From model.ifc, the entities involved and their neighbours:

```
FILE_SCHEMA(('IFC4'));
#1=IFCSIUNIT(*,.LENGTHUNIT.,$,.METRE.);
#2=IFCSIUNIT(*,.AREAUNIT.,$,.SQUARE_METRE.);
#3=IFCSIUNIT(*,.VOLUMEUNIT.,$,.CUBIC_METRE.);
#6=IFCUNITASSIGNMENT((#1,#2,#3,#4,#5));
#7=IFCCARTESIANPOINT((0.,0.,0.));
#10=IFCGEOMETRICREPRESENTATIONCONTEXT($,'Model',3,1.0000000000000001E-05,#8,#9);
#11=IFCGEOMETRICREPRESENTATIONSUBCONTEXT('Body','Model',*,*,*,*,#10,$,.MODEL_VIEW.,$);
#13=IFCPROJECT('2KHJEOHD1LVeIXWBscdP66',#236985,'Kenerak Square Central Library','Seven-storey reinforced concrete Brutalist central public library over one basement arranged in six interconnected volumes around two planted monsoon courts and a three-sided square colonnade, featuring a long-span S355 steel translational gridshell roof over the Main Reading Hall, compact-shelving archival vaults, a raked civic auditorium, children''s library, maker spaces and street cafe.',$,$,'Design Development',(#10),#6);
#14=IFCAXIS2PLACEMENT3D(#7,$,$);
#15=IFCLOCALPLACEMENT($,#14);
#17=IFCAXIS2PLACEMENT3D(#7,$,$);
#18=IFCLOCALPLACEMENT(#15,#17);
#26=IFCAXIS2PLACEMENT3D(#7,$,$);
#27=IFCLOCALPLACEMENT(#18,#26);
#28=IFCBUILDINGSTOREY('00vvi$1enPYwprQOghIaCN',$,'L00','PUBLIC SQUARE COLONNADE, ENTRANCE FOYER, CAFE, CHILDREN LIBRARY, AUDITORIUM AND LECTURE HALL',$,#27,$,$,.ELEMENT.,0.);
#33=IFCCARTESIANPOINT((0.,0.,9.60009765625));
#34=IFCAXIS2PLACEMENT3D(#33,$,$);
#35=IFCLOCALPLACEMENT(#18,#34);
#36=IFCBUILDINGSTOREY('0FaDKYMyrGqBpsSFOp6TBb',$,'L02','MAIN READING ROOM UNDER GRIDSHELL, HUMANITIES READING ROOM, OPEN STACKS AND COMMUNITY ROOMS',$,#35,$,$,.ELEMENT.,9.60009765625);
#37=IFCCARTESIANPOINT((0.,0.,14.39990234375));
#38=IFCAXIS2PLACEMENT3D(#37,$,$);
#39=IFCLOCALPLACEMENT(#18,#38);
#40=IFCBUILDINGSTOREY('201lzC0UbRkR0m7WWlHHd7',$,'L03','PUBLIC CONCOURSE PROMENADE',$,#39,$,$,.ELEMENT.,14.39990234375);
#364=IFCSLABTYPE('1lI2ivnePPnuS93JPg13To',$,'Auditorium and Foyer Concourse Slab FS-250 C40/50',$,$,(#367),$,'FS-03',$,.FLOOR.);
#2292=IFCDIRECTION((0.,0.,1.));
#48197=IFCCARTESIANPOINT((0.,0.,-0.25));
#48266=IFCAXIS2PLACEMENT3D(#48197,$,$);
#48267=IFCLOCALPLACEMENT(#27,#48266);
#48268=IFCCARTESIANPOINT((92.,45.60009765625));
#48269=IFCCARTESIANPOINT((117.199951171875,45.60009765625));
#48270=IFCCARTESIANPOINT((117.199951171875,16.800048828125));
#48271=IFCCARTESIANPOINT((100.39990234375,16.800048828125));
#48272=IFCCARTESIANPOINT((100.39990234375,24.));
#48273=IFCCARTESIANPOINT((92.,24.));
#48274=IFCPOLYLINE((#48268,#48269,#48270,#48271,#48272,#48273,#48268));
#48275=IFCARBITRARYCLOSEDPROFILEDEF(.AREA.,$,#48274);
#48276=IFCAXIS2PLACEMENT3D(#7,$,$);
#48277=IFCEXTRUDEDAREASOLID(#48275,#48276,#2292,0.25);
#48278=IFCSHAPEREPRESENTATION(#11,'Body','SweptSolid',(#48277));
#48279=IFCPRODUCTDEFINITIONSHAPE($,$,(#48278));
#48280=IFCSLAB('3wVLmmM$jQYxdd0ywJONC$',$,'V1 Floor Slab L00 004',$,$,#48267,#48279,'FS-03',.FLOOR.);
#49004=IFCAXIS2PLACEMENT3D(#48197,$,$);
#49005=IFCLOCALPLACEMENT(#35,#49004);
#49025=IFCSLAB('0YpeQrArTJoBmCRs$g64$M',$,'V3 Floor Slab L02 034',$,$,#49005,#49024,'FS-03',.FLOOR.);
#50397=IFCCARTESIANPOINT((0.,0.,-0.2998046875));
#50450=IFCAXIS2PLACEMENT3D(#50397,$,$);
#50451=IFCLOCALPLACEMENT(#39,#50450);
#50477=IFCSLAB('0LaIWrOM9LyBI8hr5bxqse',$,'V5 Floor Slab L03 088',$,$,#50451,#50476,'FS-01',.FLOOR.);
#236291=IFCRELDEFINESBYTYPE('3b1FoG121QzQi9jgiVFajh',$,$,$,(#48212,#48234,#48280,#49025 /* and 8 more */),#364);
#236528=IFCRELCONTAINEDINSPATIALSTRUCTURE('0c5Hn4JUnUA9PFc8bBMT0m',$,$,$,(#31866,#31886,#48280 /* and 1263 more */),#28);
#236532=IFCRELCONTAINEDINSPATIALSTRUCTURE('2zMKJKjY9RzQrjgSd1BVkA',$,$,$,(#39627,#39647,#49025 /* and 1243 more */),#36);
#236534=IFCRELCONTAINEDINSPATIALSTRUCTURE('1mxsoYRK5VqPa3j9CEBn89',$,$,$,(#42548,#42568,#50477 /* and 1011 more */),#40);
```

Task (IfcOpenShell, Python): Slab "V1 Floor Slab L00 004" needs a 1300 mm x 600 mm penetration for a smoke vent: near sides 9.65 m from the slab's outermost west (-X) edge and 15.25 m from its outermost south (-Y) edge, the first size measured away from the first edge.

```python
import numpy as np
import ifcopenshell
import ifcopenshell.api.feature
import ifcopenshell.api.geometry
import ifcopenshell.api.root
import ifcopenshell.geom
import ifcopenshell.util.placement
import ifcopenshell.util.representation
import ifcopenshell.util.shape
import ifcopenshell.util.unit

model = ifcopenshell.open("model.ifc")
unit_scale = ifcopenshell.util.unit.calculate_unit_scale(model)
settings = ifcopenshell.geom.settings()


def volume(element):
    """Net volume in cubic metres, openings subtracted."""
    shape = ifcopenshell.geom.create_shape(settings, element)
    return ifcopenshell.util.shape.get_volume(shape.geometry)


slab = model.by_guid("3wVLmmM$jQYxdd0ywJONC$")
before = volume(slab)

# Extent in the slab's own axes, in metres. The edges named are its -X and -Y sides.
slab_shape = ifcopenshell.geom.create_shape(settings, slab)
vertices = ifcopenshell.util.shape.get_vertices(slab_shape.geometry)
x_min, y_min, bottom = vertices.min(axis=0)
top = vertices[:, 2].max()

opening = ifcopenshell.api.root.create_entity(model, ifc_class="IfcOpeningElement", name="Smoke vent opening", predefined_type="OPENING")
context = ifcopenshell.util.representation.get_context(model, "Model", "Body", "MODEL_VIEW")
width, depth = 1.3, 0.6
outline = [(0.0, 0.0), (width, 0.0), (width, depth), (0.0, depth), (0.0, 0.0)]
# Overshoot both faces by 50 mm so the cut is clean.
shape = ifcopenshell.api.geometry.add_slab_representation(
    model, context=context, depth=top - bottom + 0.1, polyline=outline
)
ifcopenshell.api.geometry.assign_representation(model, product=opening, representation=shape)

matrix = ifcopenshell.util.placement.get_local_placement(slab.ObjectPlacement)
matrix[:, 3] = matrix @ np.append(np.array([x_min + 9.65, y_min + 15.25, bottom - 0.05]) / unit_scale, 1.0)
ifcopenshell.api.geometry.edit_object_placement(model, product=opening, matrix=matrix, is_si=False)
ifcopenshell.api.feature.add_feature(model, feature=opening, element=slab)

after = volume(slab)

print(f"slab volume {before:.3f} -> {after:.3f} m3")

model.write("model_updated.ifc")
```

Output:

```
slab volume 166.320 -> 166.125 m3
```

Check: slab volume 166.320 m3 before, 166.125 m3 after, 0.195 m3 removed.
